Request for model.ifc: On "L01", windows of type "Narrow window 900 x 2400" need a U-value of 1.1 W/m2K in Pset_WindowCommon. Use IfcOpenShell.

First a look at what the model holds.

```python
import ifcopenshell
import ifcopenshell.util.element

model = ifcopenshell.open("model.ifc")
print(model.schema)
storey = next(s for s in model.by_type("IfcBuildingStorey") if s.Name == "L01")
windows = [e for e in ifcopenshell.util.element.get_decomposition(storey) if e.is_a("IfcWindow")]
seen = {}
for e in windows:
    element_type = ifcopenshell.util.element.get_type(e)
    key = (element_type.Name if element_type != e and element_type else None, ifcopenshell.util.element.get_pset(e, "Pset_WindowCommon", "ThermalTransmittance"))
    seen[key] = seen.get(key, 0) + 1
for (name, value), count in sorted(seen.items(), key=str):
    print(count, "x", name, "|", value)
```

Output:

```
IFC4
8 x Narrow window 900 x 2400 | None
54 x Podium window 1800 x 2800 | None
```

```python
import ifcopenshell
import ifcopenshell.api.pset
import ifcopenshell.util.element

model = ifcopenshell.open("model.ifc")

storey = next(s for s in model.by_type("IfcBuildingStorey") if s.Name == "L01")
windows = [e for e in ifcopenshell.util.element.get_decomposition(storey) if e.is_a("IfcWindow")]

count = 0
for e in windows:
    element_type = ifcopenshell.util.element.get_type(e)
    if element_type in (None, e) or element_type.Name != "Narrow window 900 x 2400":
        continue
    found = ifcopenshell.util.element.get_pset(e, "Pset_WindowCommon", should_inherit=False)
    if found:
        pset = model.by_id(found["id"])
        if len(ifcopenshell.util.element.get_elements_by_pset(pset)) > 1:
            pset = ifcopenshell.api.pset.unshare_pset(model, products=[e], pset=pset)[0]
    else:
        pset = ifcopenshell.api.pset.add_pset(model, product=e, name="Pset_WindowCommon")
    ifcopenshell.api.pset.edit_pset(model, pset=pset, properties={"ThermalTransmittance": 1.1})
    count += 1

print(count, "windows updated")

model.write("model-out.ifc")
```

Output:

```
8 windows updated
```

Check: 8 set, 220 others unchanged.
